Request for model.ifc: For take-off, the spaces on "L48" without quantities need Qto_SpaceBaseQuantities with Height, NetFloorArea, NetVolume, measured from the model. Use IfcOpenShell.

First a look at what the model holds.

```python
import ifcopenshell
import ifcopenshell.util.element
import ifcopenshell.util.unit

model = ifcopenshell.open("model.ifc")
print(model.schema)
for unit_type in ("LENGTHUNIT", "AREAUNIT", "VOLUMEUNIT"):
    print(unit_type, ifcopenshell.util.unit.calculate_unit_scale(model, unit_type))
storey = next(s for s in model.by_type("IfcBuildingStorey") if s.Name == "L48")
spaces = [e for e in ifcopenshell.util.element.get_decomposition(storey) if e.is_a("IfcSpace")]
for e in sorted(spaces, key=lambda e: e.id()):
    print(e.id(), e.is_a(), e.Name, list(ifcopenshell.util.element.get_psets(e, qtos_only=True)), sep=" | ")
```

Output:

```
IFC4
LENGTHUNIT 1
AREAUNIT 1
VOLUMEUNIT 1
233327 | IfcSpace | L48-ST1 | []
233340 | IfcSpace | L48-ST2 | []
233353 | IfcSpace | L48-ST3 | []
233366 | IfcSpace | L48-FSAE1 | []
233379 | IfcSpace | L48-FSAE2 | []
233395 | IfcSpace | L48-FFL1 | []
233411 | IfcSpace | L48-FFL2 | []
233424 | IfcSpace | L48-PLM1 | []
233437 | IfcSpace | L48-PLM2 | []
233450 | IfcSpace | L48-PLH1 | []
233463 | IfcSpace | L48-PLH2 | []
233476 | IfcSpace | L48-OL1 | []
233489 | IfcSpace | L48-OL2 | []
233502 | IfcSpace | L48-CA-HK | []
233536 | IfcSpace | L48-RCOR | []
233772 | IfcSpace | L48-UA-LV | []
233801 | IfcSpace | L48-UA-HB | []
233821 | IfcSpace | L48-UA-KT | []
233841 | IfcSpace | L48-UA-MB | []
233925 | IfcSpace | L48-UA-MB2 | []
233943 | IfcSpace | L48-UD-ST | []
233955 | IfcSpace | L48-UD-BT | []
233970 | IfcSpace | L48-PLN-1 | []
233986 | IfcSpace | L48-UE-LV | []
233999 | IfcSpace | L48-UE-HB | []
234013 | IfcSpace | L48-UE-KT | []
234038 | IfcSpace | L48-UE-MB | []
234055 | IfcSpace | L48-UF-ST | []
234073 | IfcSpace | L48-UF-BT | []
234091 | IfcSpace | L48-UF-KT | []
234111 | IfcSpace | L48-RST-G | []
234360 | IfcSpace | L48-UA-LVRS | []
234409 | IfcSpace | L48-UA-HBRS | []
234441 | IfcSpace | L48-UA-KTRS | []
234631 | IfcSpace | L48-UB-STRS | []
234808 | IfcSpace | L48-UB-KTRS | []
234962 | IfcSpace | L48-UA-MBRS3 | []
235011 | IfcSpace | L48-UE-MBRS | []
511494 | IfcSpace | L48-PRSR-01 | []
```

```python
import ifcopenshell
import ifcopenshell.api.pset
import ifcopenshell.geom
import ifcopenshell.util.element
import ifcopenshell.util.shape
import ifcopenshell.util.unit

model = ifcopenshell.open("model.ifc")
unit_scale = ifcopenshell.util.unit.calculate_unit_scale(model)
area_scale = ifcopenshell.util.unit.calculate_unit_scale(model, "AREAUNIT")
volume_scale = ifcopenshell.util.unit.calculate_unit_scale(model, "VOLUMEUNIT")
settings = ifcopenshell.geom.settings()

storey = next(s for s in model.by_type("IfcBuildingStorey") if s.Name == "L48")
spaces = [e for e in ifcopenshell.util.element.get_decomposition(storey) if e.is_a("IfcSpace")]

for e in sorted(spaces, key=lambda e: e.id()):
    if ifcopenshell.util.element.get_psets(e, qtos_only=True, should_inherit=False):
        continue
    # Geometry comes back in metres, in the element's own axes.
    shape = ifcopenshell.geom.create_shape(settings, e)
    values = {
        "Height": ifcopenshell.util.shape.get_z(shape.geometry) / unit_scale,
        "NetFloorArea": ifcopenshell.util.shape.get_footprint_area(shape.geometry) / area_scale,
        "NetVolume": ifcopenshell.util.shape.get_volume(shape.geometry) / volume_scale,
    }
    qto = ifcopenshell.api.pset.add_qto(model, product=e, name="Qto_SpaceBaseQuantities")
    ifcopenshell.api.pset.edit_qto(model, qto=qto, properties=values)
    print(e.id(), {k: round(v, 3) for k, v in values.items()})

model.write("model_updated.ifc")
```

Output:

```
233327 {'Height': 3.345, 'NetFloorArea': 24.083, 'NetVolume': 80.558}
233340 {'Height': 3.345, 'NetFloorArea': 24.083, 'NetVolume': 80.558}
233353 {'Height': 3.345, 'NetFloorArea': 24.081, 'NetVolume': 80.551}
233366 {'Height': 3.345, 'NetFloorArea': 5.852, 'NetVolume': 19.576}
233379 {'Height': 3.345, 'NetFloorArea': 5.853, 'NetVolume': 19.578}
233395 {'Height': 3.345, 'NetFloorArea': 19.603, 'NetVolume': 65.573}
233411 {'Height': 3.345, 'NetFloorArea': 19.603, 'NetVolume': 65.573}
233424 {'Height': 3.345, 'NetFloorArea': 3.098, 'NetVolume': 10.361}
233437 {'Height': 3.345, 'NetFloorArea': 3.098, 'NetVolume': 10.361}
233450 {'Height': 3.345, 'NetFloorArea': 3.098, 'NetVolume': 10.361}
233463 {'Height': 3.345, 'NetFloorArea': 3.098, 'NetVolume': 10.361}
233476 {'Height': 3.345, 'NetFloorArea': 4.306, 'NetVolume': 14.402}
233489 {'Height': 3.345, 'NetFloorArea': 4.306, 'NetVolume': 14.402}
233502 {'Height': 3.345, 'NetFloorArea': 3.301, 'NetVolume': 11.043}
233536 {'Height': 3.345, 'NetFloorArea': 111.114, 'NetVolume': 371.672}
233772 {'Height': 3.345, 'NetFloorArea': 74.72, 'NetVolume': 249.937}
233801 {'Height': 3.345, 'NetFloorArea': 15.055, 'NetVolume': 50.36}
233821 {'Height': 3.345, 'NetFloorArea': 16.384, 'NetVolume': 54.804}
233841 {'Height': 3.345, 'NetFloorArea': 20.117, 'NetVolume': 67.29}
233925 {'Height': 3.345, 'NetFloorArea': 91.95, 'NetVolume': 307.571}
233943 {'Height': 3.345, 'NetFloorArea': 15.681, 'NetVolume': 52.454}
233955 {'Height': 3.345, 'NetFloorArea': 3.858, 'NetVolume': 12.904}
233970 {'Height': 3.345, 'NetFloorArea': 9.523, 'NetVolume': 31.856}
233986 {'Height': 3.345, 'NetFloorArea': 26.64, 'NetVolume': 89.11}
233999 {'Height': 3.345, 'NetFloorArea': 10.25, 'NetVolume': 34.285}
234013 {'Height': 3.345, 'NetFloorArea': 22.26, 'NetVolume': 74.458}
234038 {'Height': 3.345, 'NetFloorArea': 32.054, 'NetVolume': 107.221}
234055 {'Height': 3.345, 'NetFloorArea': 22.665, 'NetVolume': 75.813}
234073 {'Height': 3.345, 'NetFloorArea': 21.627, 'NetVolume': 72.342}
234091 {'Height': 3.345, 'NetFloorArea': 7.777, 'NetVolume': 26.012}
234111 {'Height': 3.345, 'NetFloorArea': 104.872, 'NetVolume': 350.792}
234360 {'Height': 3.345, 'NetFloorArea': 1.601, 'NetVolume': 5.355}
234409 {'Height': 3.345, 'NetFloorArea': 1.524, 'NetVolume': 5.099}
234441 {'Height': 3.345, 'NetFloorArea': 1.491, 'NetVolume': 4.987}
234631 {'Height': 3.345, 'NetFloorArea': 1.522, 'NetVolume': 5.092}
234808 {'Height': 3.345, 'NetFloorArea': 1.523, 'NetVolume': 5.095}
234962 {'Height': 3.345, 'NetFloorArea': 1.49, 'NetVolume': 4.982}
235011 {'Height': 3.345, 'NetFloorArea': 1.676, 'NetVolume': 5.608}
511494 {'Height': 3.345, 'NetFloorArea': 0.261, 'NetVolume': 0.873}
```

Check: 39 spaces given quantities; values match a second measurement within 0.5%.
